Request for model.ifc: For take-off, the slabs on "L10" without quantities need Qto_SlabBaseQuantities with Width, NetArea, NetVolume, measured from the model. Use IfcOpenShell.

First a look at what the model holds.

```python
import ifcopenshell
import ifcopenshell.util.element
import ifcopenshell.util.unit

model = ifcopenshell.open("model.ifc")
print(model.schema)
for unit_type in ("LENGTHUNIT", "AREAUNIT", "VOLUMEUNIT"):
    print(unit_type, ifcopenshell.util.unit.calculate_unit_scale(model, unit_type))
storey = next(s for s in model.by_type("IfcBuildingStorey") if s.Name == "L10")
slabs = [e for e in ifcopenshell.util.element.get_decomposition(storey) if e.is_a("IfcSlab")]
for e in sorted(slabs, key=lambda e: e.id()):
    print(e.id(), e.is_a(), e.Name, list(ifcopenshell.util.element.get_psets(e, qtos_only=True)), sep=" | ")
```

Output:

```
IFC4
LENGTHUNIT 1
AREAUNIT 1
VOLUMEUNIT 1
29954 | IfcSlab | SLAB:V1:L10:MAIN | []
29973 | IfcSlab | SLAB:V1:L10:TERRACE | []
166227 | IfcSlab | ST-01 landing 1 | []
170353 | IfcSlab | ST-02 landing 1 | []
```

```python
import ifcopenshell
import ifcopenshell.api.pset
import ifcopenshell.geom
import ifcopenshell.util.element
import ifcopenshell.util.shape
import ifcopenshell.util.unit

model = ifcopenshell.open("model.ifc")
unit_scale = ifcopenshell.util.unit.calculate_unit_scale(model)
area_scale = ifcopenshell.util.unit.calculate_unit_scale(model, "AREAUNIT")
volume_scale = ifcopenshell.util.unit.calculate_unit_scale(model, "VOLUMEUNIT")
settings = ifcopenshell.geom.settings()

storey = next(s for s in model.by_type("IfcBuildingStorey") if s.Name == "L10")
slabs = [e for e in ifcopenshell.util.element.get_decomposition(storey) if e.is_a("IfcSlab")]

for e in sorted(slabs, key=lambda e: e.id()):
    if ifcopenshell.util.element.get_psets(e, qtos_only=True, should_inherit=False):
        continue
    # Geometry comes back in metres, in the element's own axes.
    shape = ifcopenshell.geom.create_shape(settings, e)
    values = {
        "Width": ifcopenshell.util.shape.get_z(shape.geometry) / unit_scale,
        "NetArea": ifcopenshell.util.shape.get_footprint_area(shape.geometry) / area_scale,
        "NetVolume": ifcopenshell.util.shape.get_volume(shape.geometry) / volume_scale,
    }
    qto = ifcopenshell.api.pset.add_qto(model, product=e, name="Qto_SlabBaseQuantities")
    ifcopenshell.api.pset.edit_qto(model, qto=qto, properties=values)
    print(e.id(), {k: round(v, 3) for k, v in values.items()})

model.write("model_v2.ifc")
```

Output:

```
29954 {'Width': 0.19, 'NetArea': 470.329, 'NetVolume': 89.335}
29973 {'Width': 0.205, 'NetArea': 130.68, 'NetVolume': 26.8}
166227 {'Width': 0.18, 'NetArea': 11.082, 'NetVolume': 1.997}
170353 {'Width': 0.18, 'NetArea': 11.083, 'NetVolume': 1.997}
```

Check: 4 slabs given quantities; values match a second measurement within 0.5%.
